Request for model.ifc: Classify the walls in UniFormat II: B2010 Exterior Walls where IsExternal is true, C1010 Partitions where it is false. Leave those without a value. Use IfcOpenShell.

First a look at what the model holds.

```python
import ifcopenshell
import ifcopenshell.util.element

model = ifcopenshell.open("model.ifc")
print(model.schema)
print("classifications:", [c.Name for c in model.by_type("IfcClassification")])
values = [ifcopenshell.util.element.get_pset(e, "Pset_WallCommon", "IsExternal") for e in model.by_type("IfcWall")]
for value in (True, False, None):
    print("IsExternal", value, values.count(value))
```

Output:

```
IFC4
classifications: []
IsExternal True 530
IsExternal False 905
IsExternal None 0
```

```python
import ifcopenshell
import ifcopenshell.api.classification
import ifcopenshell.util.element

model = ifcopenshell.open("model.ifc")

system = ifcopenshell.api.classification.add_classification(model, classification="UniFormat II")

walls = model.by_type("IfcWall")
external = {e: ifcopenshell.util.element.get_pset(e, "Pset_WallCommon", "IsExternal") for e in walls}
for flag, code, name in ((True, "B2010", "Exterior Walls"), (False, "C1010", "Partitions")):
    products = [e for e in walls if external[e] is flag]
    ifcopenshell.api.classification.add_reference(
        model, products=products, classification=system, identification=code, name=name
    )
    print(code, len(products))

model.write("model_updated.ifc")
```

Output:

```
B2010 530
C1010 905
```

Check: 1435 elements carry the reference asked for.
